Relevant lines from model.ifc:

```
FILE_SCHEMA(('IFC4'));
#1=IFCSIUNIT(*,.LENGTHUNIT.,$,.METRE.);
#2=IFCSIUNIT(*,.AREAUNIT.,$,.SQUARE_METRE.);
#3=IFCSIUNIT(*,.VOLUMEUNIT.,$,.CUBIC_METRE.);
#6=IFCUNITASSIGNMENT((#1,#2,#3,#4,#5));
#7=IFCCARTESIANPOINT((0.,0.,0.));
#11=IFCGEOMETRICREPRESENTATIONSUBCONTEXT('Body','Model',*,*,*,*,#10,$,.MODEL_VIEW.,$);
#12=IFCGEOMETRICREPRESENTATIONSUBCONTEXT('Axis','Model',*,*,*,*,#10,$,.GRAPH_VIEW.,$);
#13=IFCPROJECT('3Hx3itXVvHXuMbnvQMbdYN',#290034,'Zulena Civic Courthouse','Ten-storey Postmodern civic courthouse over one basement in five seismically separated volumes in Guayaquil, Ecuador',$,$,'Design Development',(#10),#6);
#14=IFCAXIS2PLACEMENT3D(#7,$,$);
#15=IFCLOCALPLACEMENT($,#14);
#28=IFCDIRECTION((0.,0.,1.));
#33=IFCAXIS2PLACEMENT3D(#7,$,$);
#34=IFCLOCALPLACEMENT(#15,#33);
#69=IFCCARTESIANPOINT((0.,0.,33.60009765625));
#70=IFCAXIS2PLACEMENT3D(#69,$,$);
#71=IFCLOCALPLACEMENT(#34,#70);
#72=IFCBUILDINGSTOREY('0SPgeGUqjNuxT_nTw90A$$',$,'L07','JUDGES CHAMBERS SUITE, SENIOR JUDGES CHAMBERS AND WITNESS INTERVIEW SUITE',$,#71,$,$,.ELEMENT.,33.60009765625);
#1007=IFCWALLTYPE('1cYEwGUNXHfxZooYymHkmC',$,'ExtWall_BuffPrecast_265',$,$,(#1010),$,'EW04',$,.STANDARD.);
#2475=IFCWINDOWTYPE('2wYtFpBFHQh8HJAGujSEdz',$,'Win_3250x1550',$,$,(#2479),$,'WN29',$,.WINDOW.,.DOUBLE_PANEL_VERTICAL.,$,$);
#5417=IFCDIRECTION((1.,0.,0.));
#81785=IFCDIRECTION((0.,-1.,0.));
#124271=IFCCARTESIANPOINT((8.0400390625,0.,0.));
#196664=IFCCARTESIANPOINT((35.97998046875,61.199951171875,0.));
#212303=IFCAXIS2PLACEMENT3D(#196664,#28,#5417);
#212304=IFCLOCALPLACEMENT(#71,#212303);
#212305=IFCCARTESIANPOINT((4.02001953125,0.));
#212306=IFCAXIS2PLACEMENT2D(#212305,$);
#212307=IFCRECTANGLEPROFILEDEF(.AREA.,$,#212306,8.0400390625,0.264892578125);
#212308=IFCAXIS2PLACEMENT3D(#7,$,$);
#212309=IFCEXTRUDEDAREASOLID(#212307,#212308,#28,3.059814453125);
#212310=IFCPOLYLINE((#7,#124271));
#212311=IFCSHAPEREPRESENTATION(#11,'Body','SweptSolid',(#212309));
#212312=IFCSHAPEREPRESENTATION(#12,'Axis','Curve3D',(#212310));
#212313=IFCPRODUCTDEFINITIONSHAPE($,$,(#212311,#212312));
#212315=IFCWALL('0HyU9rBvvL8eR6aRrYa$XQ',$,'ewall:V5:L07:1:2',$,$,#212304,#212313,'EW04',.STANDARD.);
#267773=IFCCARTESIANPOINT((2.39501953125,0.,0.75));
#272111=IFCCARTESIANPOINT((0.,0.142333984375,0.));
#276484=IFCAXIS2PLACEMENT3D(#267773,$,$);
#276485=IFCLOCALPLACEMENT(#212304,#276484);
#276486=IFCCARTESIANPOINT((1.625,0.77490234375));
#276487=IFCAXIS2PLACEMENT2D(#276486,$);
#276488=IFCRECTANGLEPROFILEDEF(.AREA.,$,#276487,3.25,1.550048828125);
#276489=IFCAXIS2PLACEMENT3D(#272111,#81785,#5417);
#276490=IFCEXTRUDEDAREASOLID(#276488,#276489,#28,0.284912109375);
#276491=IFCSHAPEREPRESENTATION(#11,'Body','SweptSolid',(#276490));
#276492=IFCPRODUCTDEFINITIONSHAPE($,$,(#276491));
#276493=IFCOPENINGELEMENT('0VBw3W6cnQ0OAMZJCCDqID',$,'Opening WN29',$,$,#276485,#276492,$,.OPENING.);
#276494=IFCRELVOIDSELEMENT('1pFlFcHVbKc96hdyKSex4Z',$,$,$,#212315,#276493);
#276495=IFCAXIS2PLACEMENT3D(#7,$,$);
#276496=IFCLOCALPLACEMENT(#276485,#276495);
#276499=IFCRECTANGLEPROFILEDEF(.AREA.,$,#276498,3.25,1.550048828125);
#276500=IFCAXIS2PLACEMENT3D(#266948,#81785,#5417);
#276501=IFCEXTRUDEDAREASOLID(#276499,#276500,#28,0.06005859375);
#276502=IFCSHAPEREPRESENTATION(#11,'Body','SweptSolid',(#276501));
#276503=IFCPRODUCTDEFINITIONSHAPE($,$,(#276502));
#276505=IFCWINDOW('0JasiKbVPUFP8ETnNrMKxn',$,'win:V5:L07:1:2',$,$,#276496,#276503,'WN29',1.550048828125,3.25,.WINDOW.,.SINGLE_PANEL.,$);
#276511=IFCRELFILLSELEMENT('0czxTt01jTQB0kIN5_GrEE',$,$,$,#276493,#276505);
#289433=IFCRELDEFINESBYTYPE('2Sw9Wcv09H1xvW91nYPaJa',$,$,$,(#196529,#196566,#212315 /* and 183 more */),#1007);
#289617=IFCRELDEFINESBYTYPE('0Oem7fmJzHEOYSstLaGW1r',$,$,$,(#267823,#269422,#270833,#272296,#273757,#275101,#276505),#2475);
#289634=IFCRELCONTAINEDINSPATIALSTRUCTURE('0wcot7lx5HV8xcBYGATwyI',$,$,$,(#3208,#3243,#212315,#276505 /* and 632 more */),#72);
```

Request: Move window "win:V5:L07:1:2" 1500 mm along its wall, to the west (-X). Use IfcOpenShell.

```python
import ifcopenshell
import ifcopenshell.api.geometry
import ifcopenshell.util.placement
import ifcopenshell.util.unit

model = ifcopenshell.open("model.ifc")
unit_scale = ifcopenshell.util.unit.calculate_unit_scale(model)

window = model.by_guid("0JasiKbVPUFP8ETnNrMKxn")
opening = window.FillsVoids[0].RelatingOpeningElement
wall = opening.VoidsElements[0].RelatingBuildingElement

wall_matrix = ifcopenshell.util.placement.get_local_placement(wall.ObjectPlacement)
shift = wall_matrix[:3, 0] * -1.5 / unit_scale
before = ifcopenshell.util.placement.get_local_placement(window.ObjectPlacement)[:3, 3].copy()

# The window is placed relative to its opening, so it follows when the opening moves.
matrix = ifcopenshell.util.placement.get_local_placement(opening.ObjectPlacement)
matrix[:3, 3] += shift
ifcopenshell.api.geometry.edit_object_placement(
    model, product=opening, matrix=matrix, is_si=False, should_transform_children=True
)

after = ifcopenshell.util.placement.get_local_placement(window.ObjectPlacement)[:3, 3]
print("window moved by", (after - before).round(3) + 0.0)

model.write("model_v2.ifc")
```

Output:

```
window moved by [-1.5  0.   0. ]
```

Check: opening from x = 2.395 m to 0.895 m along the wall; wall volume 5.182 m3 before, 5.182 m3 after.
